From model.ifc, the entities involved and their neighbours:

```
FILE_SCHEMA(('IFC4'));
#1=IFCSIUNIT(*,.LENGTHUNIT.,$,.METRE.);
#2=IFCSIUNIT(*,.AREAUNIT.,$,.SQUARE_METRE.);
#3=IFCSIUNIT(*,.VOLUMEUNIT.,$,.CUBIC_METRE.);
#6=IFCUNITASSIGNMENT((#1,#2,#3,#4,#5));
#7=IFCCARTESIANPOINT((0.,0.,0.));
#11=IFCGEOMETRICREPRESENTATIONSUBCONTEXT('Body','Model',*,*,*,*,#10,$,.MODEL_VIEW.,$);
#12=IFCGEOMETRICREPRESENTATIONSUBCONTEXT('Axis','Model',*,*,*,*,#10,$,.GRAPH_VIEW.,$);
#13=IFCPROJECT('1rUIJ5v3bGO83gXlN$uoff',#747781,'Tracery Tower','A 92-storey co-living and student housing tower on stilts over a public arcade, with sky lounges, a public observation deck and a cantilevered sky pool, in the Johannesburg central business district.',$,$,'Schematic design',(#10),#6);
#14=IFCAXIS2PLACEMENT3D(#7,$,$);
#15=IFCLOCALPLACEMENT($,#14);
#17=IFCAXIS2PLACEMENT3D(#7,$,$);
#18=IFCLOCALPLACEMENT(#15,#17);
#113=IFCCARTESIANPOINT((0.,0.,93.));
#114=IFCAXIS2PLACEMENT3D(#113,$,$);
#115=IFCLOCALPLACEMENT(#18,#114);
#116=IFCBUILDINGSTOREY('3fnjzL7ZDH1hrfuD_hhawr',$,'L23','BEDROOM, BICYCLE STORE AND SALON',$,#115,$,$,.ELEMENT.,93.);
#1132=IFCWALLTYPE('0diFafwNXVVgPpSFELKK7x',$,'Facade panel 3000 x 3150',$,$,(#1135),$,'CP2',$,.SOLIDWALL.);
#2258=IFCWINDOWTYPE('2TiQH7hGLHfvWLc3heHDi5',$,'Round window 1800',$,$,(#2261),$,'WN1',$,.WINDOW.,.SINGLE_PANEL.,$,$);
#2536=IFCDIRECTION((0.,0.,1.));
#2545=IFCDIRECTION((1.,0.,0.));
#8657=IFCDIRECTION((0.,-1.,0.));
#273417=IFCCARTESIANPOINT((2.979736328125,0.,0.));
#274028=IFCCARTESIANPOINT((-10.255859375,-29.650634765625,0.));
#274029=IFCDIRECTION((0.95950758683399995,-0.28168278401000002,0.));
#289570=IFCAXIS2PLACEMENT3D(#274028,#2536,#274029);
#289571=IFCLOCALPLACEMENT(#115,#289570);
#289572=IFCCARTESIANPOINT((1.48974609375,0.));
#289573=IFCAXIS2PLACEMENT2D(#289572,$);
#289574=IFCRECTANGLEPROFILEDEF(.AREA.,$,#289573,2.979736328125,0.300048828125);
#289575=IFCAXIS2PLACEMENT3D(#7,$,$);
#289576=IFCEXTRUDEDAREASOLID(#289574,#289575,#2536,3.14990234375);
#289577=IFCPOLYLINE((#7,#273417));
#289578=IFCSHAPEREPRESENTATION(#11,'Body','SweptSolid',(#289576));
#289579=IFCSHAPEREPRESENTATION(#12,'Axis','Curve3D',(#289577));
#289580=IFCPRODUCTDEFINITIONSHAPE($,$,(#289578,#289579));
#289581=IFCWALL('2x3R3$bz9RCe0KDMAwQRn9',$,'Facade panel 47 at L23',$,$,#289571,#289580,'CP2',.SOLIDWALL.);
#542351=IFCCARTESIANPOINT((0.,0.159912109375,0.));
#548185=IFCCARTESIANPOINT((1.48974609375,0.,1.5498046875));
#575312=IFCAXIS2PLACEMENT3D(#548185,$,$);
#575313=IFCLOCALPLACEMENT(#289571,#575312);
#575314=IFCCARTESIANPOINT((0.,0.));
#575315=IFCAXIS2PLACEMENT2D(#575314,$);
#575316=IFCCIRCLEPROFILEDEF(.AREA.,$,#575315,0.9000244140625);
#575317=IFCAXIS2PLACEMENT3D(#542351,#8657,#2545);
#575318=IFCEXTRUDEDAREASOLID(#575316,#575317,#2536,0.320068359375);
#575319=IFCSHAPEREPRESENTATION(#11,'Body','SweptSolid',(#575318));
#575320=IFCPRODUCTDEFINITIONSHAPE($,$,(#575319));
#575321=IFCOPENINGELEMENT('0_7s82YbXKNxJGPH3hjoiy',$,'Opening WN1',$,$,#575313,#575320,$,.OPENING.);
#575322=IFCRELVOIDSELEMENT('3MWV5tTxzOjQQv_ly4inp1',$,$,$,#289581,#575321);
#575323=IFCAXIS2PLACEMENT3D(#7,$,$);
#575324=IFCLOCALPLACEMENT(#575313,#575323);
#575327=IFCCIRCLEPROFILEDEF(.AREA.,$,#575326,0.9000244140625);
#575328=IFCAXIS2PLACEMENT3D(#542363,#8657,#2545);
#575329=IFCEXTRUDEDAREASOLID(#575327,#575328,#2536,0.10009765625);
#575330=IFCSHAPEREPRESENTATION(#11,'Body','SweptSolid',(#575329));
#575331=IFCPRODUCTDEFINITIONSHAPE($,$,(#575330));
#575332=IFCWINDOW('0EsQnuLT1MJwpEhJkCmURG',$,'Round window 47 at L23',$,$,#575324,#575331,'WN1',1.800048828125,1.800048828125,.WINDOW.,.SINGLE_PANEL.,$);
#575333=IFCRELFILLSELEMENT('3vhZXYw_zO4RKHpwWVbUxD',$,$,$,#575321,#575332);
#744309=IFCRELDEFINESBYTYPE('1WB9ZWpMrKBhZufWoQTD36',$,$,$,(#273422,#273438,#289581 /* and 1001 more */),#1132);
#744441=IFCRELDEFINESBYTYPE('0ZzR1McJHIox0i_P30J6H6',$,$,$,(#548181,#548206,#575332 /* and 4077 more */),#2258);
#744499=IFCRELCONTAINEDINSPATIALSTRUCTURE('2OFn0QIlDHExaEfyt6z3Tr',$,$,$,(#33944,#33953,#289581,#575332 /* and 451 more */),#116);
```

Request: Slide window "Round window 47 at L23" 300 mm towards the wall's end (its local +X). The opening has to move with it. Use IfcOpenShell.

```python
import ifcopenshell
import ifcopenshell.api.geometry
import ifcopenshell.util.placement
import ifcopenshell.util.unit

model = ifcopenshell.open("model.ifc")
unit_scale = ifcopenshell.util.unit.calculate_unit_scale(model)

window = model.by_id(575332)
opening = window.FillsVoids[0].RelatingOpeningElement
wall = opening.VoidsElements[0].RelatingBuildingElement

wall_matrix = ifcopenshell.util.placement.get_local_placement(wall.ObjectPlacement)
shift = wall_matrix[:3, 0] * 0.3 / unit_scale
before = ifcopenshell.util.placement.get_local_placement(window.ObjectPlacement)[:3, 3].copy()

# The window is placed relative to its opening, so it follows when the opening moves.
matrix = ifcopenshell.util.placement.get_local_placement(opening.ObjectPlacement)
matrix[:3, 3] += shift
ifcopenshell.api.geometry.edit_object_placement(
    model, product=opening, matrix=matrix, is_si=False, should_transform_children=True
)

after = ifcopenshell.util.placement.get_local_placement(window.ObjectPlacement)[:3, 3]
print("window moved by", (after - before).round(3) + 0.0)

model.write("model_rev.ifc")
```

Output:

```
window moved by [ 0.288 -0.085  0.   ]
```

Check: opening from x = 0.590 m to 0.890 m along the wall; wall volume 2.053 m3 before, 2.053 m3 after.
